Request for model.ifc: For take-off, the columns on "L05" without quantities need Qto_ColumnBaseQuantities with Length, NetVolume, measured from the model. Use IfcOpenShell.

First a look at what the model holds.

```python
import ifcopenshell
import ifcopenshell.util.element
import ifcopenshell.util.unit

model = ifcopenshell.open("model.ifc")
print(model.schema)
for unit_type in ("LENGTHUNIT", "AREAUNIT", "VOLUMEUNIT"):
    print(unit_type, ifcopenshell.util.unit.calculate_unit_scale(model, unit_type))
storey = next(s for s in model.by_type("IfcBuildingStorey") if s.Name == "L05")
columns = [e for e in ifcopenshell.util.element.get_decomposition(storey) if e.is_a("IfcColumn")]
for e in sorted(columns, key=lambda e: e.id()):
    print(e.id(), e.is_a(), e.Name, list(ifcopenshell.util.element.get_psets(e, qtos_only=True)), sep=" | ")
```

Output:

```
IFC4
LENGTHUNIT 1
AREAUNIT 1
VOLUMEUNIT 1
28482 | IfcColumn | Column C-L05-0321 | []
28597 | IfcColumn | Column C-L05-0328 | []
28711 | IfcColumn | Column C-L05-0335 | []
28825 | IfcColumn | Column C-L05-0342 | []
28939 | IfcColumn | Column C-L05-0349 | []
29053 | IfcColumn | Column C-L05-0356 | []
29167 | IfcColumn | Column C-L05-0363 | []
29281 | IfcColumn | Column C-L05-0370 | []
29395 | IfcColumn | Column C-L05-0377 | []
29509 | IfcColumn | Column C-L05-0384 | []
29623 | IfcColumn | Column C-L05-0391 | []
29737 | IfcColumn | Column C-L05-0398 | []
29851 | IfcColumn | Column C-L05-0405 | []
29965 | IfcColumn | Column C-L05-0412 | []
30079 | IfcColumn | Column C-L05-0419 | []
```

```python
import ifcopenshell
import ifcopenshell.api.pset
import ifcopenshell.geom
import ifcopenshell.util.element
import ifcopenshell.util.shape
import ifcopenshell.util.unit

model = ifcopenshell.open("model.ifc")
unit_scale = ifcopenshell.util.unit.calculate_unit_scale(model)
volume_scale = ifcopenshell.util.unit.calculate_unit_scale(model, "VOLUMEUNIT")
settings = ifcopenshell.geom.settings()

storey = next(s for s in model.by_type("IfcBuildingStorey") if s.Name == "L05")
columns = [e for e in ifcopenshell.util.element.get_decomposition(storey) if e.is_a("IfcColumn")]

for e in sorted(columns, key=lambda e: e.id()):
    if ifcopenshell.util.element.get_psets(e, qtos_only=True, should_inherit=False):
        continue
    # Geometry comes back in metres, in the element's own axes.
    shape = ifcopenshell.geom.create_shape(settings, e)
    values = {
        "Length": ifcopenshell.util.shape.get_z(shape.geometry) / unit_scale,
        "NetVolume": ifcopenshell.util.shape.get_volume(shape.geometry) / volume_scale,
    }
    qto = ifcopenshell.api.pset.add_qto(model, product=e, name="Qto_ColumnBaseQuantities")
    ifcopenshell.api.pset.edit_qto(model, qto=qto, properties=values)
    print(e.id(), {k: round(v, 3) for k, v in values.items()})

model.write("model_v2.ifc")
```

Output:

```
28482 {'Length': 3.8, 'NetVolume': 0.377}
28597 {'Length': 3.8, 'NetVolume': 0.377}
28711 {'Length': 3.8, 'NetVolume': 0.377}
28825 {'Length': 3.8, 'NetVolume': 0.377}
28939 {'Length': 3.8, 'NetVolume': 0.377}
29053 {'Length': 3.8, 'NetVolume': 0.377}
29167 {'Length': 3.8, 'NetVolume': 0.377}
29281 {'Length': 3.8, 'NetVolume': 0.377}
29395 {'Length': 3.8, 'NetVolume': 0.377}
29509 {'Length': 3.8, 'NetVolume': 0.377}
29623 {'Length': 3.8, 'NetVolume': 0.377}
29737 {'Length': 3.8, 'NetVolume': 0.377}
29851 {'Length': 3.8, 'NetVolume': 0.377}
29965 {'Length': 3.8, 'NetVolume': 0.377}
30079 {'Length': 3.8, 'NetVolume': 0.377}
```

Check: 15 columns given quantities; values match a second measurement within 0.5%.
